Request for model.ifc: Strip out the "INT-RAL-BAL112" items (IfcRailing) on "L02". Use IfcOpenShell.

First a look at what the model holds.

```python
import ifcopenshell
import ifcopenshell.util.element

model = ifcopenshell.open("model.ifc")
print(model.schema)
storey = next(s for s in model.by_type("IfcBuildingStorey") if s.Name == "L02")
railings = [e for e in ifcopenshell.util.element.get_decomposition(storey) if e.is_a("IfcRailing")]
seen = {}
for e in railings:
    element_type = ifcopenshell.util.element.get_type(e)
    name = element_type.Name if element_type not in (None, e) else None
    seen[name] = seen.get(name, 0) + 1
for name, count in sorted(seen.items(), key=str):
    print(count, "x", name)
```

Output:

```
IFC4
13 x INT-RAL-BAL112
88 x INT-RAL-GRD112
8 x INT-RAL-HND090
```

```python
import ifcopenshell
import ifcopenshell.api.root
import ifcopenshell.util.element

model = ifcopenshell.open("model.ifc")

storey = next(s for s in model.by_type("IfcBuildingStorey") if s.Name == "L02")
railings = [e for e in ifcopenshell.util.element.get_decomposition(storey) if e.is_a("IfcRailing")]
targets = [e for e in railings if (t := ifcopenshell.util.element.get_type(e)) not in (None, e) and t.Name == "INT-RAL-BAL112"]

for e in targets:
    ifcopenshell.api.root.remove_product(model, product=e)
print(len(targets), "removed")

model.write("model_updated.ifc")
```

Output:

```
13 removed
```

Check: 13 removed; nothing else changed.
